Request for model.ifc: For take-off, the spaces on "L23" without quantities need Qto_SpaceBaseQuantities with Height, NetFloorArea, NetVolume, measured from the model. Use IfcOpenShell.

First a look at what the model holds.

```python
import ifcopenshell
import ifcopenshell.util.element
import ifcopenshell.util.unit

model = ifcopenshell.open("model.ifc")
print(model.schema)
for unit_type in ("LENGTHUNIT", "AREAUNIT", "VOLUMEUNIT"):
    print(unit_type, ifcopenshell.util.unit.calculate_unit_scale(model, unit_type))
storey = next(s for s in model.by_type("IfcBuildingStorey") if s.Name == "L23")
spaces = [e for e in ifcopenshell.util.element.get_decomposition(storey) if e.is_a("IfcSpace")]
for e in sorted(spaces, key=lambda e: e.id()):
    print(e.id(), e.is_a(), e.Name, list(ifcopenshell.util.element.get_psets(e, qtos_only=True)), sep=" | ")
```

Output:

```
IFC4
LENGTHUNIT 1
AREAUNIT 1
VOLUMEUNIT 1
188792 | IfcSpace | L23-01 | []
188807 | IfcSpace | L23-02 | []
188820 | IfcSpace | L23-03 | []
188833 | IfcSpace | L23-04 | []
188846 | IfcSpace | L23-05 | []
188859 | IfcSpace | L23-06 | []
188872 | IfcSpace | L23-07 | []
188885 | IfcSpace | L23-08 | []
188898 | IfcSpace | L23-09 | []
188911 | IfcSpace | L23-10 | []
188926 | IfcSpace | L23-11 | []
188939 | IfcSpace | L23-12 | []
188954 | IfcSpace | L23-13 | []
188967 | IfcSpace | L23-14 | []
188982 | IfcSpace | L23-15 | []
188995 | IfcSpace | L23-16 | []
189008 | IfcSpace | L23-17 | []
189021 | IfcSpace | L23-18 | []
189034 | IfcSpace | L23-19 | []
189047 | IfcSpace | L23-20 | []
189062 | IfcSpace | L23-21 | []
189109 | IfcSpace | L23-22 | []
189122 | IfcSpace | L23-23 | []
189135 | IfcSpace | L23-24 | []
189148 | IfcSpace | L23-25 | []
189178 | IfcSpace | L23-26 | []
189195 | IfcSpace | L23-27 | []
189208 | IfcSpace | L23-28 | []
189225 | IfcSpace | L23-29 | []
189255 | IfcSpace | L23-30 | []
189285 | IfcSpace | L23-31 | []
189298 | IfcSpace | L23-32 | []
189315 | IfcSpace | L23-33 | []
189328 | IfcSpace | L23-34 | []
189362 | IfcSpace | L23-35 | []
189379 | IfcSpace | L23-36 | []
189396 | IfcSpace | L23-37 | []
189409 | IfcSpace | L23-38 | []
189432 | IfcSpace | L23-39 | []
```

```python
import ifcopenshell
import ifcopenshell.api.pset
import ifcopenshell.geom
import ifcopenshell.util.element
import ifcopenshell.util.shape
import ifcopenshell.util.unit

model = ifcopenshell.open("model.ifc")
unit_scale = ifcopenshell.util.unit.calculate_unit_scale(model)
area_scale = ifcopenshell.util.unit.calculate_unit_scale(model, "AREAUNIT")
volume_scale = ifcopenshell.util.unit.calculate_unit_scale(model, "VOLUMEUNIT")
settings = ifcopenshell.geom.settings()

storey = next(s for s in model.by_type("IfcBuildingStorey") if s.Name == "L23")
spaces = [e for e in ifcopenshell.util.element.get_decomposition(storey) if e.is_a("IfcSpace")]

for e in sorted(spaces, key=lambda e: e.id()):
    if ifcopenshell.util.element.get_psets(e, qtos_only=True, should_inherit=False):
        continue
    # Geometry comes back in metres, in the element's own axes.
    shape = ifcopenshell.geom.create_shape(settings, e)
    values = {
        "Height": ifcopenshell.util.shape.get_z(shape.geometry) / unit_scale,
        "NetFloorArea": ifcopenshell.util.shape.get_footprint_area(shape.geometry) / area_scale,
        "NetVolume": ifcopenshell.util.shape.get_volume(shape.geometry) / volume_scale,
    }
    qto = ifcopenshell.api.pset.add_qto(model, product=e, name="Qto_SpaceBaseQuantities")
    ifcopenshell.api.pset.edit_qto(model, qto=qto, properties=values)
    print(e.id(), {k: round(v, 3) for k, v in values.items()})

model.write("model_rev.ifc")
```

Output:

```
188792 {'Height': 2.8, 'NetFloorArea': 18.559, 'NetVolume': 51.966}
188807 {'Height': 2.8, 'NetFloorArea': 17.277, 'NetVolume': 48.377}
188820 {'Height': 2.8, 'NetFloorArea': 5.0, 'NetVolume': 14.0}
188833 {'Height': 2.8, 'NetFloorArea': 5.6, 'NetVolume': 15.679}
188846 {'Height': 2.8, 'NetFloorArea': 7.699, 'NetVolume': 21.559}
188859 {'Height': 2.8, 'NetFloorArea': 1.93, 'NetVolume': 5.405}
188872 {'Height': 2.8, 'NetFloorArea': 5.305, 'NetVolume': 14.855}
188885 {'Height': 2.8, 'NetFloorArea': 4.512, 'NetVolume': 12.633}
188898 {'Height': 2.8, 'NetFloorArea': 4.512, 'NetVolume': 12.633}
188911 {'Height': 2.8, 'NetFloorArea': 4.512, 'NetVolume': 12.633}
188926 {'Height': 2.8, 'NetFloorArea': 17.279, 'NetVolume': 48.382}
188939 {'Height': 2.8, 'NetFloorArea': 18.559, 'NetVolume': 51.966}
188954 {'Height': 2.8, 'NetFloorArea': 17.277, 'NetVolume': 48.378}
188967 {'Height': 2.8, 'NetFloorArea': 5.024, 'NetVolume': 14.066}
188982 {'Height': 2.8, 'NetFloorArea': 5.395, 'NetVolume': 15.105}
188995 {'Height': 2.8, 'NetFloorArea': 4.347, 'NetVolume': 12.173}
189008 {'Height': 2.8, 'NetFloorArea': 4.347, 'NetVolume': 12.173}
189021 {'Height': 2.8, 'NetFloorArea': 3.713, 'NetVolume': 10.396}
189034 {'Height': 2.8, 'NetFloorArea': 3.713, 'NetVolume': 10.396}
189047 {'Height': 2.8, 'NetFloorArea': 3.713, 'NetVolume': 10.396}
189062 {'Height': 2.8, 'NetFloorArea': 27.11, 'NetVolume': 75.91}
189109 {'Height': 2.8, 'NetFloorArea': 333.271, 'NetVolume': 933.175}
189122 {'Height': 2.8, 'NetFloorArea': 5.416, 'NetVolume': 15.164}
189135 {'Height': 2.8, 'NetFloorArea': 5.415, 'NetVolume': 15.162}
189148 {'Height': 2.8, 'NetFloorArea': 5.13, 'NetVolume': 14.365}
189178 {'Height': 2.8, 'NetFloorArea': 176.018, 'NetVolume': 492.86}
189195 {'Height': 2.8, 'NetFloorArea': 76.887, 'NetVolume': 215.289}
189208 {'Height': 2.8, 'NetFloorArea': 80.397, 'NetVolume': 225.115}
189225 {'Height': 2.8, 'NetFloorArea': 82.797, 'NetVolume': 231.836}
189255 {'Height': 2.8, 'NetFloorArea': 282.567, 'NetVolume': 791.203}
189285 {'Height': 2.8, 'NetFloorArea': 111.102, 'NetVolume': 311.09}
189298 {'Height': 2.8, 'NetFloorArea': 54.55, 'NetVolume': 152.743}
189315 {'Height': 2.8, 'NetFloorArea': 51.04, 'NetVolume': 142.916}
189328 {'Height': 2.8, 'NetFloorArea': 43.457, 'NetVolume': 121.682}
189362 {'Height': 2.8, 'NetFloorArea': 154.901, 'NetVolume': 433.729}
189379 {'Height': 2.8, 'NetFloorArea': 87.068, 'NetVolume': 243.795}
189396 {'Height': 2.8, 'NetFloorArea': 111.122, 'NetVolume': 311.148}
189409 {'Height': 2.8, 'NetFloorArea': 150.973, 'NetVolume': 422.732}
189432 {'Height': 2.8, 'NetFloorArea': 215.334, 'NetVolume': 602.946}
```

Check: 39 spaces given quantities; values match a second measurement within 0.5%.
